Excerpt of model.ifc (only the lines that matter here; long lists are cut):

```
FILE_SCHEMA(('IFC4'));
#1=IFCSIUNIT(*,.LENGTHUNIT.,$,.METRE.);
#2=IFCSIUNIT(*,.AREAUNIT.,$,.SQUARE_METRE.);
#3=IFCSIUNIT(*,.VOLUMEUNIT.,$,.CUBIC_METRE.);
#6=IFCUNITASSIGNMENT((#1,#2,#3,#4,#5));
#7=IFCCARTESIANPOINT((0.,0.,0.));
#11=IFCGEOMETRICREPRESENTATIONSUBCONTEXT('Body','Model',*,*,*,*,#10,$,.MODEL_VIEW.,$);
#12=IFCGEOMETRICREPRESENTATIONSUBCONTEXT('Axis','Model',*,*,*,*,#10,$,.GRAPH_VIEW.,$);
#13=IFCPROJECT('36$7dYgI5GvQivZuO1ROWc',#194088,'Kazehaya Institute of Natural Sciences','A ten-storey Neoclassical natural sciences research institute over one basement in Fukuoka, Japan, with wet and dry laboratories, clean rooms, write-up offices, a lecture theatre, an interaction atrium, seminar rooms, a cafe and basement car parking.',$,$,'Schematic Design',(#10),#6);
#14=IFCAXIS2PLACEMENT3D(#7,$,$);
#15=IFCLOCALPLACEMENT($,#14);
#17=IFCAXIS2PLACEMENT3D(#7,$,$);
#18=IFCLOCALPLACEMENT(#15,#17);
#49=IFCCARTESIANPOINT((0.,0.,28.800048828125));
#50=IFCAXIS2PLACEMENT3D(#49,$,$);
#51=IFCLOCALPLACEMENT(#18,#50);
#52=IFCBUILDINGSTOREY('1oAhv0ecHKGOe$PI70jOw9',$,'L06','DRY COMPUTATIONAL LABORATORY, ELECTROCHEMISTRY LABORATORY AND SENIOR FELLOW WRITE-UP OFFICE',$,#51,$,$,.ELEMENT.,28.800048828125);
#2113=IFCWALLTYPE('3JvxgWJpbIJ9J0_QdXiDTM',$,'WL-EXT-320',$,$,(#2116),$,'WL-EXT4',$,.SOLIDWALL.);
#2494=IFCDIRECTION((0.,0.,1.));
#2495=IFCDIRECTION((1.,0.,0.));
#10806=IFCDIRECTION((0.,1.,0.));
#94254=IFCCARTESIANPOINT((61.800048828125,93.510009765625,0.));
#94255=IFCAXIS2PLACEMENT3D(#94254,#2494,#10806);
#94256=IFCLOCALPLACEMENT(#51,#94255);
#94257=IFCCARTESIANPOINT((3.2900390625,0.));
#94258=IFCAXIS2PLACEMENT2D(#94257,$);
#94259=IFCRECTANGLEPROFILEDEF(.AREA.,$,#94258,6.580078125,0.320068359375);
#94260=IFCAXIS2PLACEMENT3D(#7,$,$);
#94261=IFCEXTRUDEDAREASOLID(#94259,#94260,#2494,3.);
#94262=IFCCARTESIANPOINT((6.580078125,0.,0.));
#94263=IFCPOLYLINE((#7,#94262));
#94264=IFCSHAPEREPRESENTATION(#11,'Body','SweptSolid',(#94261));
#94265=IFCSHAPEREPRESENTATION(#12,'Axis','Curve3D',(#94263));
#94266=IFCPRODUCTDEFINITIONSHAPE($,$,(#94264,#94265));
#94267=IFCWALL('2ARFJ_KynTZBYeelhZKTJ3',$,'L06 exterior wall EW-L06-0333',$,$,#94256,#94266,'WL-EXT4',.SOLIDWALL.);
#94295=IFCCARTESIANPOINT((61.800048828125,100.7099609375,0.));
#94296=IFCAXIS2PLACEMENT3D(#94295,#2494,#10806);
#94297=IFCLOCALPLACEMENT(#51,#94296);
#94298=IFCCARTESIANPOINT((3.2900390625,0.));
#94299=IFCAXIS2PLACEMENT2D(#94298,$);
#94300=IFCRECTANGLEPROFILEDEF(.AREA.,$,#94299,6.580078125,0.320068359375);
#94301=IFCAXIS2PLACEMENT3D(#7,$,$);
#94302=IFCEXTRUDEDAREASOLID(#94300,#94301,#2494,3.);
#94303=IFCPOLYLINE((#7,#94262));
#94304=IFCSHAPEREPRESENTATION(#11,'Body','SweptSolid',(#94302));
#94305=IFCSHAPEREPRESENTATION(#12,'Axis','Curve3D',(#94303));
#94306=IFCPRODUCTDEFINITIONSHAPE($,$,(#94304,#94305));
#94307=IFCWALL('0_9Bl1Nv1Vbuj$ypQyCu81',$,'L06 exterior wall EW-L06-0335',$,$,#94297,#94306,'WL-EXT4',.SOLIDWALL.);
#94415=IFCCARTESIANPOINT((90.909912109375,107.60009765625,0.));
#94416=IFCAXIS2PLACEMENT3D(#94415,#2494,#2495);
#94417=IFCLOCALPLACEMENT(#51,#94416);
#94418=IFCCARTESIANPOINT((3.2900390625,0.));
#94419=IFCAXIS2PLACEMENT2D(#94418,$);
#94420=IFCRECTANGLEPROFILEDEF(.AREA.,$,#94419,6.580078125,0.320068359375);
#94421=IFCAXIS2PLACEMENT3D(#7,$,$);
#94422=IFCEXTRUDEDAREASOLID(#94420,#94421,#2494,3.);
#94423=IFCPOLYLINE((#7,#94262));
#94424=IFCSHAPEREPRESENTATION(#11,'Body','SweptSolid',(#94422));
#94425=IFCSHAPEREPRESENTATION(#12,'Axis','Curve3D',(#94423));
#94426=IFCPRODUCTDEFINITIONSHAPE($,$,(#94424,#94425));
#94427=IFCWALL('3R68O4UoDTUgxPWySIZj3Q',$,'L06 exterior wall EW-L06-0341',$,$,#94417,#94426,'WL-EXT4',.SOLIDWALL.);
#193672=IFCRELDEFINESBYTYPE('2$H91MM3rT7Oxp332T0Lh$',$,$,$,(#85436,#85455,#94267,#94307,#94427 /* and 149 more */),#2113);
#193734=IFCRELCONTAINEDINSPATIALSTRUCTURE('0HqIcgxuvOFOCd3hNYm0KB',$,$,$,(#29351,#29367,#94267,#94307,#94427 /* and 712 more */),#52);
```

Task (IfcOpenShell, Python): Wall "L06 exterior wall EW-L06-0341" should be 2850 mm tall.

```python
import ifcopenshell
import ifcopenshell.geom
import ifcopenshell.util.representation
import ifcopenshell.util.shape
import ifcopenshell.util.unit

model = ifcopenshell.open("model.ifc")
unit_scale = ifcopenshell.util.unit.calculate_unit_scale(model)
settings = ifcopenshell.geom.settings()


def volume(element):
    """Net volume in cubic metres, openings subtracted."""
    shape = ifcopenshell.geom.create_shape(settings, element)
    return ifcopenshell.util.shape.get_volume(shape.geometry)


wall = model.by_id(94427)
before = volume(wall)

body = ifcopenshell.util.representation.get_representation(wall, "Model", "Body")
solid = body.Items[0]
old_height = solid.Depth
solid.Depth = 2.85 / unit_scale
after = volume(wall)

print(f"height {old_height:g} -> {solid.Depth:g}, volume {before:.3f} -> {after:.3f} m3")

model.write("model_v2.ifc")
```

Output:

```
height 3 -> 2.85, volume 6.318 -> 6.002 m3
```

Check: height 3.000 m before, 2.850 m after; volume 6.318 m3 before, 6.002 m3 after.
